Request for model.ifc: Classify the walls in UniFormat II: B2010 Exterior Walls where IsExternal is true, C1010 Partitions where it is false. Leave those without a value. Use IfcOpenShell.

First a look at what the model holds.

```python
import ifcopenshell
import ifcopenshell.util.element

model = ifcopenshell.open("model.ifc")
print(model.schema)
print("classifications:", [c.Name for c in model.by_type("IfcClassification")])
values = [ifcopenshell.util.element.get_pset(e, "Pset_WallCommon", "IsExternal") for e in model.by_type("IfcWall")]
for value in (True, False, None):
    print("IsExternal", value, values.count(value))
```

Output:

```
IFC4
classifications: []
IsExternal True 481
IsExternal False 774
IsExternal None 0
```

```python
import ifcopenshell
import ifcopenshell.api.classification
import ifcopenshell.util.element

model = ifcopenshell.open("model.ifc")

system = ifcopenshell.api.classification.add_classification(model, classification="UniFormat II")

walls = model.by_type("IfcWall")
external = {e: ifcopenshell.util.element.get_pset(e, "Pset_WallCommon", "IsExternal") for e in walls}
for flag, code, name in ((True, "B2010", "Exterior Walls"), (False, "C1010", "Partitions")):
    products = [e for e in walls if external[e] is flag]
    ifcopenshell.api.classification.add_reference(
        model, products=products, classification=system, identification=code, name=name
    )
    print(code, len(products))

model.write("model-out.ifc")
```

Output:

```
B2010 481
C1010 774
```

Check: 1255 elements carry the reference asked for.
